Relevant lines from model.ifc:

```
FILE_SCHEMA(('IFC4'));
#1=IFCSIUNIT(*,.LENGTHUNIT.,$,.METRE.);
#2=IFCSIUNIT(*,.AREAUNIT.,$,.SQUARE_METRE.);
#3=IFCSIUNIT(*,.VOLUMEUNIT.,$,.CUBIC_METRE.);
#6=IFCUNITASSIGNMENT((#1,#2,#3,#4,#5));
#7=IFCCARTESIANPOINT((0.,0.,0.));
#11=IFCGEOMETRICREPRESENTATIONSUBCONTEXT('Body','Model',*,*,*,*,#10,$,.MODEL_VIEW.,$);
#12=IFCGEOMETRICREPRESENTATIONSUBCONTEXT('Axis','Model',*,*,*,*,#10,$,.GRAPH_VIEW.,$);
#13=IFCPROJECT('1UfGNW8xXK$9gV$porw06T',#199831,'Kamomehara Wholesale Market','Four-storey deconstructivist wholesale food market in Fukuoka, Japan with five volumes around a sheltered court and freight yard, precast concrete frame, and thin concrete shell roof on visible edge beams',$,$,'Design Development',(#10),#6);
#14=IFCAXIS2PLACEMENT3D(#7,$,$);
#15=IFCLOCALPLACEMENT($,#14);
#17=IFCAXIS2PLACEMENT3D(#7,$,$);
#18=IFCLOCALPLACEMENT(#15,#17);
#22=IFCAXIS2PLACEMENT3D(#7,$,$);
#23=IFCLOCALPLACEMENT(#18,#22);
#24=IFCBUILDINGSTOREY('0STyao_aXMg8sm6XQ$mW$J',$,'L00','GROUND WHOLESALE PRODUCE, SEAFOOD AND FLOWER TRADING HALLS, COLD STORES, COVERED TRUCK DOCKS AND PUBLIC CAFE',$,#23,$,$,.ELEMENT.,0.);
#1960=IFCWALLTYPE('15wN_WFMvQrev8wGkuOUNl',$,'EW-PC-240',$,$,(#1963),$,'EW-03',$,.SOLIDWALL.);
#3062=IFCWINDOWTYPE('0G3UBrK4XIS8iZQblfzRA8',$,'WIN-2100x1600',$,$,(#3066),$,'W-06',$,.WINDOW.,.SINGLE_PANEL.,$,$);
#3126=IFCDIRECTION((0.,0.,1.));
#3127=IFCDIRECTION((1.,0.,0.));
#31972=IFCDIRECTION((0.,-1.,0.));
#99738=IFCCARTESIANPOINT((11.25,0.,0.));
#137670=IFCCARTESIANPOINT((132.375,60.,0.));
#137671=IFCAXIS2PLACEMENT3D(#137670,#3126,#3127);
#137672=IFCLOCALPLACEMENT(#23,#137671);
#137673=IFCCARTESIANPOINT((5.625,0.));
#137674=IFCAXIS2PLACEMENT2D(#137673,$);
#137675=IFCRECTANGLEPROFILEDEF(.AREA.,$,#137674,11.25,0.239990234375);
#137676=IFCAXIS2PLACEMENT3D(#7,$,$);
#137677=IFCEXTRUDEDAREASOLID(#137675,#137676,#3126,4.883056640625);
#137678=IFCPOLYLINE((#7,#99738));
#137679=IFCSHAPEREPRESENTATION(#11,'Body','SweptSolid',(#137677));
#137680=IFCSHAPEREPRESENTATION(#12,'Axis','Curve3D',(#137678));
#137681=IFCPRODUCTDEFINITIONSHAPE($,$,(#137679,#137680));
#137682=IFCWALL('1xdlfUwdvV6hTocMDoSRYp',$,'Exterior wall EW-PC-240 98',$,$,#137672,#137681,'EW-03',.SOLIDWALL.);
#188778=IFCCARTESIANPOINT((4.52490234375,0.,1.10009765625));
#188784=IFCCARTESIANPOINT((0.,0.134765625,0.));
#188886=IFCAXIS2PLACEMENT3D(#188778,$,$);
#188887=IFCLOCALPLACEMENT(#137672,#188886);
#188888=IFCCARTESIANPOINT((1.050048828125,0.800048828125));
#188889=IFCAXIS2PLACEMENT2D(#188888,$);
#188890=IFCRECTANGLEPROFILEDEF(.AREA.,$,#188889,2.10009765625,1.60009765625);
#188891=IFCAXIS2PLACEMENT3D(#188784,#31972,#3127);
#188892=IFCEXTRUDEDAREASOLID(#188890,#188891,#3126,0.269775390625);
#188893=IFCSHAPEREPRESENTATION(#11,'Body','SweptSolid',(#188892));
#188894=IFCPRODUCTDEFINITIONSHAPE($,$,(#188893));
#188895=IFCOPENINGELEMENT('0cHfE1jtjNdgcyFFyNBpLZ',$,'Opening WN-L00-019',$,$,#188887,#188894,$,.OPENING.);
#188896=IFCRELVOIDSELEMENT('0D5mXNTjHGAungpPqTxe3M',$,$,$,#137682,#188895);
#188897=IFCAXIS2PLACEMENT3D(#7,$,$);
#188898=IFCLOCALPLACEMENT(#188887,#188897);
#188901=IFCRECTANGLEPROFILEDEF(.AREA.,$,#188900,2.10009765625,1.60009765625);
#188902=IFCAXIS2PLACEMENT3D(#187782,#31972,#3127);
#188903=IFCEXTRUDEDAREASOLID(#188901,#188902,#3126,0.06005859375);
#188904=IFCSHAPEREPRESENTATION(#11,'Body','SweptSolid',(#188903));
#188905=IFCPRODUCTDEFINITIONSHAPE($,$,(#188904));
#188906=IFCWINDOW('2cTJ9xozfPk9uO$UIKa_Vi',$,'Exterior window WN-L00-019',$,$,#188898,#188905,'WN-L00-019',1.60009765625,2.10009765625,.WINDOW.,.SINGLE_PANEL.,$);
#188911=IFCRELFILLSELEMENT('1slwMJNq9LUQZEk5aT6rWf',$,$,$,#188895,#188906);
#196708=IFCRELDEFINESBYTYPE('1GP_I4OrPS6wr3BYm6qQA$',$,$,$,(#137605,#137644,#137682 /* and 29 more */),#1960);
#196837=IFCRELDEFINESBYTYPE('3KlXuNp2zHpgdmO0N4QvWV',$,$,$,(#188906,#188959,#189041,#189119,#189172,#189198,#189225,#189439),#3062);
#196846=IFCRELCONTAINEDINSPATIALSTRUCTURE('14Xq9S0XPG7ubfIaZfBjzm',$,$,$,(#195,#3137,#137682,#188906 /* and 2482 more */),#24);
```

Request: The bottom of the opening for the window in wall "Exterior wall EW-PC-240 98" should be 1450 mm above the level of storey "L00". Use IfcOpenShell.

```python
import numpy as np
import ifcopenshell
import ifcopenshell.api.geometry
import ifcopenshell.geom
import ifcopenshell.util.element
import ifcopenshell.util.placement
import ifcopenshell.util.shape
import ifcopenshell.util.unit

model = ifcopenshell.open("model.ifc")
unit_scale = ifcopenshell.util.unit.calculate_unit_scale(model)

window = model.by_guid("2cTJ9xozfPk9uO$UIKa_Vi")
opening = window.FillsVoids[0].RelatingOpeningElement
storey = ifcopenshell.util.element.get_container(window, ifc_class="IfcBuildingStorey")
level = ifcopenshell.util.placement.get_local_placement(storey.ObjectPlacement)[2, 3]

# The opening's origin need not be at the sill, so measure its lowest point.
shape = ifcopenshell.geom.create_shape(ifcopenshell.geom.settings(), opening)
bottom = ifcopenshell.util.shape.get_shape_bottom_elevation(shape, shape.geometry) / unit_scale
dz = level + 1.45 - bottom

shift = np.array([0.0, 0.0, dz])
# The window is placed relative to its opening, so it follows when the opening moves.
matrix = ifcopenshell.util.placement.get_local_placement(opening.ObjectPlacement)
matrix[:3, 3] += shift
ifcopenshell.api.geometry.edit_object_placement(
    model, product=opening, matrix=matrix, is_si=False, should_transform_children=True
)

print(f"moved by {dz * unit_scale:+.3f} m")

model.write("model_v2.ifc")
```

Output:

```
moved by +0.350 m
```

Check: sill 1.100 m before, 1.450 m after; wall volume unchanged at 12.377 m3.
